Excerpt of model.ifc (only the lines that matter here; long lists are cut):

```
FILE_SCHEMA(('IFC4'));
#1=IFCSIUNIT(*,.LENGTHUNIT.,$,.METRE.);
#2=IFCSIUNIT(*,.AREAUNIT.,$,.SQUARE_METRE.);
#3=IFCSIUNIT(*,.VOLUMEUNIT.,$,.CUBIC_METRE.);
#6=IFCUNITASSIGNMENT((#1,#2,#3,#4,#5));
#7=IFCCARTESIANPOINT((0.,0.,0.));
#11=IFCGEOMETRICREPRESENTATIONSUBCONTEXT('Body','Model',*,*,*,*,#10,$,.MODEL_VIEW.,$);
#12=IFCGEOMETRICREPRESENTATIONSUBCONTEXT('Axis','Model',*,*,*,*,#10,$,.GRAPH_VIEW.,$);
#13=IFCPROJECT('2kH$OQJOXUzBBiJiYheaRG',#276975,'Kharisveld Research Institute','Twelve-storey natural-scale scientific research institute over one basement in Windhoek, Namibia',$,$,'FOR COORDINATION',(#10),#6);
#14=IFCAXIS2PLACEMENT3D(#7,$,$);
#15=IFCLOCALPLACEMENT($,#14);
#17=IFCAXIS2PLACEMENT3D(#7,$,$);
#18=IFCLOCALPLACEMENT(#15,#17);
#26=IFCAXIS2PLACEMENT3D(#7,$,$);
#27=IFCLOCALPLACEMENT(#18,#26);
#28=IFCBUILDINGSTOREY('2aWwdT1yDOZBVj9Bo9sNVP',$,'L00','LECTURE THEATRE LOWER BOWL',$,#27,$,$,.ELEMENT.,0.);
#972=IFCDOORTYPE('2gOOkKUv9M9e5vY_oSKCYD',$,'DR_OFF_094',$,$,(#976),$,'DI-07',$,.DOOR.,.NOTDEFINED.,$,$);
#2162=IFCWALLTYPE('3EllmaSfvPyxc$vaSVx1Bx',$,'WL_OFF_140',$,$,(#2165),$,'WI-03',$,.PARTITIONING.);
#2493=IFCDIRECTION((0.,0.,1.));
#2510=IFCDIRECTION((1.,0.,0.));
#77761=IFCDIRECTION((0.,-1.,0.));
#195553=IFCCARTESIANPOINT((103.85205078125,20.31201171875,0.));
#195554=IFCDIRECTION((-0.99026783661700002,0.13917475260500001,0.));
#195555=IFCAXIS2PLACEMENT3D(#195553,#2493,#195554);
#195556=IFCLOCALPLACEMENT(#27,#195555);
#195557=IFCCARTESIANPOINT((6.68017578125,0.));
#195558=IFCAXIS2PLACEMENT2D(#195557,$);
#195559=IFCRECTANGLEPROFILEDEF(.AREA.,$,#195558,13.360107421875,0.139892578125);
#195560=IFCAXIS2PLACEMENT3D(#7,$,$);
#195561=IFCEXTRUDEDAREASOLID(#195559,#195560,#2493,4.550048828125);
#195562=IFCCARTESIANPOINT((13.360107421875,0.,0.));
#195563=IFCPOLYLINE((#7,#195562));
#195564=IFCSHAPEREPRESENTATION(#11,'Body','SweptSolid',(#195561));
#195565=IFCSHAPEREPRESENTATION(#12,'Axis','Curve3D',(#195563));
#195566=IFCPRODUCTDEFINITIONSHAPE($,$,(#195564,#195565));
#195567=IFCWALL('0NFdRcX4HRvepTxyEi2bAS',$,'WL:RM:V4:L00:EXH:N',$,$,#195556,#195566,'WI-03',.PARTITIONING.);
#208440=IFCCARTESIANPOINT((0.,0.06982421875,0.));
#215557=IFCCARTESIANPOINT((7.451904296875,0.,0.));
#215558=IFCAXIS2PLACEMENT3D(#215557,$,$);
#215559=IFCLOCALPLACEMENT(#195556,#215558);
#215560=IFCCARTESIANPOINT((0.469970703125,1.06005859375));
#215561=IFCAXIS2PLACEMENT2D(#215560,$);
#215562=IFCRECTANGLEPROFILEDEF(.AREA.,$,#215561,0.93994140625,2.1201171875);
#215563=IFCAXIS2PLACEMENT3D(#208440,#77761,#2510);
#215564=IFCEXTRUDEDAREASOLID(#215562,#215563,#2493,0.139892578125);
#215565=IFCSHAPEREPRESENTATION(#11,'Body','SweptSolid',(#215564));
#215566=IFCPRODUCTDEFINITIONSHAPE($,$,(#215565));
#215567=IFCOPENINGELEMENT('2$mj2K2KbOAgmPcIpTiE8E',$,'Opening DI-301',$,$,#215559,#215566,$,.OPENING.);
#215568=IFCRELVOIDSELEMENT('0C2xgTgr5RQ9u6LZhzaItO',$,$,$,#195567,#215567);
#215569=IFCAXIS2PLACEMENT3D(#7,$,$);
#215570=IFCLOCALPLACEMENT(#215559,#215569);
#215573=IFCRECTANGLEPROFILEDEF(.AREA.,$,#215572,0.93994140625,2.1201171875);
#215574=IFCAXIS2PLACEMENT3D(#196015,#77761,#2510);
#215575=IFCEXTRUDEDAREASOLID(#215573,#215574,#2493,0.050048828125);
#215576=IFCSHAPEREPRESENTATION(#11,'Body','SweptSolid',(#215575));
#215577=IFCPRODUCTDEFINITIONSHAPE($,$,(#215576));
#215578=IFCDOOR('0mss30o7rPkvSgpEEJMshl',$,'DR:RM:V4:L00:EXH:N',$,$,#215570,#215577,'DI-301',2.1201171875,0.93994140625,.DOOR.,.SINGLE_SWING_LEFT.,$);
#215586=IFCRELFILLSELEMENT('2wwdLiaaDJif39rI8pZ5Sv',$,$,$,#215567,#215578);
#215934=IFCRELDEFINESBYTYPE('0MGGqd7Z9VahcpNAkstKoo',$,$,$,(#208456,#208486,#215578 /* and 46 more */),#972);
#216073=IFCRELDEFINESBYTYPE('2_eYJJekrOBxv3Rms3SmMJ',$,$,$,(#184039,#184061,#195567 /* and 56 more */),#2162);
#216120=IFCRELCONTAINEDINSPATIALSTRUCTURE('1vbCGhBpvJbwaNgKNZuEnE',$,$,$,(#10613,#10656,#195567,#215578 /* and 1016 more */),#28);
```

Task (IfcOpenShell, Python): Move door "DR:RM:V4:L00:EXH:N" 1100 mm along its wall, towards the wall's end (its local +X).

```python
import ifcopenshell
import ifcopenshell.api.geometry
import ifcopenshell.util.placement

model = ifcopenshell.open("model.ifc")

door = model.by_id(215578)
opening = door.FillsVoids[0].RelatingOpeningElement
wall = opening.VoidsElements[0].RelatingBuildingElement

wall_matrix = ifcopenshell.util.placement.get_local_placement(wall.ObjectPlacement)
shift = wall_matrix[:3, 0] * 1.1
before = ifcopenshell.util.placement.get_local_placement(door.ObjectPlacement)[:3, 3].copy()

# The door is placed relative to its opening, so it follows when the opening moves.
matrix = ifcopenshell.util.placement.get_local_placement(opening.ObjectPlacement)
matrix[:3, 3] += shift
ifcopenshell.api.geometry.edit_object_placement(
    model, product=opening, matrix=matrix, is_si=False, should_transform_children=True
)

after = ifcopenshell.util.placement.get_local_placement(door.ObjectPlacement)[:3, 3]
print("door moved by", (after - before).round(3) + 0.0)

model.write("model_edited.ifc")
```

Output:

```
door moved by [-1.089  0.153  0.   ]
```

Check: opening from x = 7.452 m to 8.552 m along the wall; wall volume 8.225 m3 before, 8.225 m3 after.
